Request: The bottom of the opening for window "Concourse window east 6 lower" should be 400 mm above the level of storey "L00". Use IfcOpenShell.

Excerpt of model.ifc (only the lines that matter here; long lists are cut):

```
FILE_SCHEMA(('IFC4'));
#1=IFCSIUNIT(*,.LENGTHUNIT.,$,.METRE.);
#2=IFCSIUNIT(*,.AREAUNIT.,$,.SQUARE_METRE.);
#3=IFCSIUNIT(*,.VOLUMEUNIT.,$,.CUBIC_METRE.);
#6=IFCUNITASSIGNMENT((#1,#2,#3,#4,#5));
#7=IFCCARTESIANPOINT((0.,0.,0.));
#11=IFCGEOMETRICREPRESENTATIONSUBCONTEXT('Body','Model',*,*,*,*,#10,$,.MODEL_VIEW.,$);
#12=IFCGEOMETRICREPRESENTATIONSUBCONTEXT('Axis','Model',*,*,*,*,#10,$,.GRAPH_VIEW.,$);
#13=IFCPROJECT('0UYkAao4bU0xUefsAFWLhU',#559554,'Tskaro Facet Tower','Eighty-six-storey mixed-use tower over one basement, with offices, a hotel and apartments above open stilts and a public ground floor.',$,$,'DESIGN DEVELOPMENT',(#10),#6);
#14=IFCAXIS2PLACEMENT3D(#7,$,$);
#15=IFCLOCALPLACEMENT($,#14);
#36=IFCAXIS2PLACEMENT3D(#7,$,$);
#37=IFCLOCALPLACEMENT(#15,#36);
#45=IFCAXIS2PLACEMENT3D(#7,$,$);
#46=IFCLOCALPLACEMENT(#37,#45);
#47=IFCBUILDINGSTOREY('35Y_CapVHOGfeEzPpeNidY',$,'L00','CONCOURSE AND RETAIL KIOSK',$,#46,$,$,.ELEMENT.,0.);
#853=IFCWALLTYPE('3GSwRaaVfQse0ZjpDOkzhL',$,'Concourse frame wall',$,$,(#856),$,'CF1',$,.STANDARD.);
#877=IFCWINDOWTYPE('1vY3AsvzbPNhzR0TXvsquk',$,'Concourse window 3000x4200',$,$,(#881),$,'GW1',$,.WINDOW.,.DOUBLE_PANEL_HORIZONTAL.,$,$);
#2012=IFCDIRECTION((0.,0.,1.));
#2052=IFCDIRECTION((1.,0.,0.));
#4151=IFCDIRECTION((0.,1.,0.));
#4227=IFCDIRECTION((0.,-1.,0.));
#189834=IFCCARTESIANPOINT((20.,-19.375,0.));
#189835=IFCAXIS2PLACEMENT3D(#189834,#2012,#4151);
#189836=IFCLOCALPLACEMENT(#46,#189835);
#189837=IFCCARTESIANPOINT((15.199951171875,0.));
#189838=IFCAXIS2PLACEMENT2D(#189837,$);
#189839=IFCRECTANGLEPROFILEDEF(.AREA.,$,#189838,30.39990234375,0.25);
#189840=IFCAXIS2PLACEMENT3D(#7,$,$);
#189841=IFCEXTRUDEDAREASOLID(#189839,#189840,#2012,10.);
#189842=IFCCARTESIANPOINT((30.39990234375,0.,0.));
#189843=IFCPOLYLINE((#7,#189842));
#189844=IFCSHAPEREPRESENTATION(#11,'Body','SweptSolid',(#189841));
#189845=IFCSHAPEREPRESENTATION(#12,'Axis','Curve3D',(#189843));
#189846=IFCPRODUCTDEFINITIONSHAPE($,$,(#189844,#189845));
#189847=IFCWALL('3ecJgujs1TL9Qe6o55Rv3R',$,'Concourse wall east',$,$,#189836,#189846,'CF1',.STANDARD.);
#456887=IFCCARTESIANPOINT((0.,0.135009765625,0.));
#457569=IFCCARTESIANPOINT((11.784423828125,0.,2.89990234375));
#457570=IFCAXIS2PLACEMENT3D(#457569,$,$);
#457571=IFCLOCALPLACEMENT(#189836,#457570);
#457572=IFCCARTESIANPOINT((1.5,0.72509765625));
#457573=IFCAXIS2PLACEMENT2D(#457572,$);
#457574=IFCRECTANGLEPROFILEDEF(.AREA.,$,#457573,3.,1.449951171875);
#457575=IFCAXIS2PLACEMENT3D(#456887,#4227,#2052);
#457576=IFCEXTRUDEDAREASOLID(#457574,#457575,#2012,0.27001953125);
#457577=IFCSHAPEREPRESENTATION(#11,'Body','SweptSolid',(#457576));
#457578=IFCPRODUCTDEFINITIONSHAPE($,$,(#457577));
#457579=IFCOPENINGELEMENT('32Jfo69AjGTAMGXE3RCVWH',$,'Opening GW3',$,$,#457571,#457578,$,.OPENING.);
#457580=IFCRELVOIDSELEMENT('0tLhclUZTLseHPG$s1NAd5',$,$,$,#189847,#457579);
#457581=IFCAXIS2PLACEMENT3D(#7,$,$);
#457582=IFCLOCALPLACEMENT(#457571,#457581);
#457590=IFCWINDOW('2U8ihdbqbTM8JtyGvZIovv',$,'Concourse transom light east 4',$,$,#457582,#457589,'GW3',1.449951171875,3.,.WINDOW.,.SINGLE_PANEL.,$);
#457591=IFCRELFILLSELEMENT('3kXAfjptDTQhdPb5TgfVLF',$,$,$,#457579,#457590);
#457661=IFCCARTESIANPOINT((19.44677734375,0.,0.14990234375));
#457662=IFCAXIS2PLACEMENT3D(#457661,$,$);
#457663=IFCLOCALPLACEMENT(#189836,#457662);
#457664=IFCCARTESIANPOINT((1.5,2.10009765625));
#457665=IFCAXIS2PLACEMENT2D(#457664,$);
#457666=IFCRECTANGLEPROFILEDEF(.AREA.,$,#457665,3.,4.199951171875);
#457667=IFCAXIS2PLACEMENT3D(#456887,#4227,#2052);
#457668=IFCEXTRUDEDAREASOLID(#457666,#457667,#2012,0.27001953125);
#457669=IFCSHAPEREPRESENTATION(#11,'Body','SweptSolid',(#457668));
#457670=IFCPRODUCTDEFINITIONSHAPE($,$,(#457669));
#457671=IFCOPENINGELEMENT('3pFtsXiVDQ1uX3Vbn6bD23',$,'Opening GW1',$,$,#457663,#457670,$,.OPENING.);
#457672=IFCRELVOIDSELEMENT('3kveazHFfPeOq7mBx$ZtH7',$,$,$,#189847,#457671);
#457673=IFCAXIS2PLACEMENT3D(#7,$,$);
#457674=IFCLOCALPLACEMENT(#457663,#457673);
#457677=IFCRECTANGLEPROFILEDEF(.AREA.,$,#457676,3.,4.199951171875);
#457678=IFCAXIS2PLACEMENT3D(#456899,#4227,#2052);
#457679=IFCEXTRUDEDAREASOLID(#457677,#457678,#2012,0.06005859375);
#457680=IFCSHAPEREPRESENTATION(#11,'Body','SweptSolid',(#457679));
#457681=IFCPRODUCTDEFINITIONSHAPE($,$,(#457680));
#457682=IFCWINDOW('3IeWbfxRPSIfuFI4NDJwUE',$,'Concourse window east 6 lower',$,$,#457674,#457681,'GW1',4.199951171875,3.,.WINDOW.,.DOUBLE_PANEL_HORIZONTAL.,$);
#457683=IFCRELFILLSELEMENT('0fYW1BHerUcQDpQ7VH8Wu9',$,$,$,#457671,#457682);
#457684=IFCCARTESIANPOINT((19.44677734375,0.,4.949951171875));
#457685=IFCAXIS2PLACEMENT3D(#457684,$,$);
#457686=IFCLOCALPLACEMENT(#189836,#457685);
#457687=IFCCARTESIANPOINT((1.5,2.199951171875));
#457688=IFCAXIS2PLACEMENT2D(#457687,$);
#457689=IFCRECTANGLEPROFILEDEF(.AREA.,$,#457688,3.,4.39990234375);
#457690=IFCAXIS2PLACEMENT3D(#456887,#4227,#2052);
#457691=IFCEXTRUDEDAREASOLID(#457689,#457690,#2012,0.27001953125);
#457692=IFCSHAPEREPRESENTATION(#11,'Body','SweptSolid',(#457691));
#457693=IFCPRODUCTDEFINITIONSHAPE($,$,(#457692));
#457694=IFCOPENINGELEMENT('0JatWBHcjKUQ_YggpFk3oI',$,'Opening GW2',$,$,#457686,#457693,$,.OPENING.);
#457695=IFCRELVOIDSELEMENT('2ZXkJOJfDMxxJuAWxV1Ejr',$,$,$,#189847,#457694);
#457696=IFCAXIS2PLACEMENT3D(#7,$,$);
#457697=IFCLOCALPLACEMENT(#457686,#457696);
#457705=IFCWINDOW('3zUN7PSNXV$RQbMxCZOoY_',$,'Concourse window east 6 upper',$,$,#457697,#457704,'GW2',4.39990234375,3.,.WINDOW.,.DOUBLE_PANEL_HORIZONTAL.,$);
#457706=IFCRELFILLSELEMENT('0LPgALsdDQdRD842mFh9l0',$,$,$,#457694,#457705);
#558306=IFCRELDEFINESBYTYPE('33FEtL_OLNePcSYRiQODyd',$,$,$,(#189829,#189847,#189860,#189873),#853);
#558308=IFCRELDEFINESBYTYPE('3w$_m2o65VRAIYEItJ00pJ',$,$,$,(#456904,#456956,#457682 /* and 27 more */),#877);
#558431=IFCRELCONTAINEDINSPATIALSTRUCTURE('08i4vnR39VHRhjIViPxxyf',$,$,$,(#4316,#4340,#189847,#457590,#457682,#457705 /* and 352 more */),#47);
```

```python
import numpy as np
import ifcopenshell
import ifcopenshell.api.geometry
import ifcopenshell.geom
import ifcopenshell.util.element
import ifcopenshell.util.placement
import ifcopenshell.util.shape
import ifcopenshell.util.unit

model = ifcopenshell.open("model.ifc")
unit_scale = ifcopenshell.util.unit.calculate_unit_scale(model)

window = model.by_guid("3IeWbfxRPSIfuFI4NDJwUE")
opening = window.FillsVoids[0].RelatingOpeningElement
storey = ifcopenshell.util.element.get_container(window, ifc_class="IfcBuildingStorey")
level = ifcopenshell.util.placement.get_local_placement(storey.ObjectPlacement)[2, 3]

# The opening's origin need not be at the sill, so measure its lowest point.
shape = ifcopenshell.geom.create_shape(ifcopenshell.geom.settings(), opening)
bottom = ifcopenshell.util.shape.get_shape_bottom_elevation(shape, shape.geometry) / unit_scale
dz = level + 0.4 / unit_scale - bottom

shift = np.array([0.0, 0.0, dz])
# The window is placed relative to its opening, so it follows when the opening moves.
matrix = ifcopenshell.util.placement.get_local_placement(opening.ObjectPlacement)
matrix[:3, 3] += shift
ifcopenshell.api.geometry.edit_object_placement(
    model, product=opening, matrix=matrix, is_si=False, should_transform_children=True
)

print(f"moved by {dz * unit_scale:+.3f} m")

model.write("model_rev.ifc")
```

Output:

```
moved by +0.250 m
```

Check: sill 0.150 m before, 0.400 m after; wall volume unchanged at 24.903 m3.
